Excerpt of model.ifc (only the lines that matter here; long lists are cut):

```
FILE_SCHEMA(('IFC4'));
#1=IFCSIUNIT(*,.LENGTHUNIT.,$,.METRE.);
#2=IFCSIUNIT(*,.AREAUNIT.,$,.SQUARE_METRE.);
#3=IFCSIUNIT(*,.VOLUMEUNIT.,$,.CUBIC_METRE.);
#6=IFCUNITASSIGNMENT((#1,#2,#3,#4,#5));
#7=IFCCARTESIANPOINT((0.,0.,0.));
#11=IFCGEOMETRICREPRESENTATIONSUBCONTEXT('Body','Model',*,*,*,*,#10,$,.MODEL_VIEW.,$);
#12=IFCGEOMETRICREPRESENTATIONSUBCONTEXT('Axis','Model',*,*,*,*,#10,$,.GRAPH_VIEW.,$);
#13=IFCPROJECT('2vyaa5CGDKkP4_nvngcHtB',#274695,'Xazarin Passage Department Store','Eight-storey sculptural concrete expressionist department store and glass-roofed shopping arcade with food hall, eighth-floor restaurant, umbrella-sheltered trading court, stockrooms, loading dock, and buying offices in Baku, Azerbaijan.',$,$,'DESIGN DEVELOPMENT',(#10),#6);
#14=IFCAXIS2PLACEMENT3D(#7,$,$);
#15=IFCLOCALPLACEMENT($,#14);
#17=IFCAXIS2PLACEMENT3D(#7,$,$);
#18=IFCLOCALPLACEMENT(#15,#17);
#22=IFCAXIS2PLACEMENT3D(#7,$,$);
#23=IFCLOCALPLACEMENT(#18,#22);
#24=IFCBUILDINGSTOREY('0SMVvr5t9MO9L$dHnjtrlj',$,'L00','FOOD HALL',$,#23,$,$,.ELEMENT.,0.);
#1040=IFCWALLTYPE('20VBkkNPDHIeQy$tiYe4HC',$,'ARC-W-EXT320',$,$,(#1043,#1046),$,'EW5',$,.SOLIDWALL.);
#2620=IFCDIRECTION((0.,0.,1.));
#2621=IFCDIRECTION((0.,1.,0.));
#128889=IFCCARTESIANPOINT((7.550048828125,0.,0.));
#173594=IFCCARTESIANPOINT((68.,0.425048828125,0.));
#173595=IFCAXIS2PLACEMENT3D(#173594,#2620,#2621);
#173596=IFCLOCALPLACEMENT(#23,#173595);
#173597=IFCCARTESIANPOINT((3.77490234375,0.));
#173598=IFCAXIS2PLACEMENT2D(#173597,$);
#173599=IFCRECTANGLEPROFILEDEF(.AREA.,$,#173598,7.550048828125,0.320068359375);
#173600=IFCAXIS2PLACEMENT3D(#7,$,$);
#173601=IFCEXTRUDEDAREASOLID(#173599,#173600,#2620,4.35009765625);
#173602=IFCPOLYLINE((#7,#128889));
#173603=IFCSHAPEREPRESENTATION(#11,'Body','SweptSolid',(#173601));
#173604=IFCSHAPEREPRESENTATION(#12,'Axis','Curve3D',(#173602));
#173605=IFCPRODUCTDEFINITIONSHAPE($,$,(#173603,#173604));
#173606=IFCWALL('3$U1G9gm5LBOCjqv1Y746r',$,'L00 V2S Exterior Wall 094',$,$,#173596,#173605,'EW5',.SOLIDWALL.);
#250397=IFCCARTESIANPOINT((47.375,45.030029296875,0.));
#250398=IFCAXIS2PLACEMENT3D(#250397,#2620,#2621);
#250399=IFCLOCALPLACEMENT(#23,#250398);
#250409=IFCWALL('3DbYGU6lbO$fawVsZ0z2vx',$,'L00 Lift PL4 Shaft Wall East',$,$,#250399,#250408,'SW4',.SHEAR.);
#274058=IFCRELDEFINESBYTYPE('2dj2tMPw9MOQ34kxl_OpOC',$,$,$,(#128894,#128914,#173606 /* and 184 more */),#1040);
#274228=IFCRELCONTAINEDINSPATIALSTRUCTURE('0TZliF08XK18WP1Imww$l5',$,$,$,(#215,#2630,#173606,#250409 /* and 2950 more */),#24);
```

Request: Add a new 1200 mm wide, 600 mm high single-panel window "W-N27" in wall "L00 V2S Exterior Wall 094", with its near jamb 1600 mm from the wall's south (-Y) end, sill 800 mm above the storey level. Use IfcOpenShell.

```python
import numpy as np
import ifcopenshell
import ifcopenshell.api.feature
import ifcopenshell.api.geometry
import ifcopenshell.api.root
import ifcopenshell.api.spatial
import ifcopenshell.geom
import ifcopenshell.util.element
import ifcopenshell.util.placement
import ifcopenshell.util.representation
import ifcopenshell.util.shape
import ifcopenshell.util.unit

model = ifcopenshell.open("model.ifc")
unit_scale = ifcopenshell.util.unit.calculate_unit_scale(model)
settings = ifcopenshell.geom.settings()


def volume(element):
    """Net volume in cubic metres, openings subtracted."""
    shape = ifcopenshell.geom.create_shape(settings, element)
    return ifcopenshell.util.shape.get_volume(shape.geometry)


wall = model.by_id(173606)
storey = ifcopenshell.util.element.get_container(wall, ifc_class="IfcBuildingStorey")
context = ifcopenshell.util.representation.get_context(model, "Model", "Body", "MODEL_VIEW")
before = volume(wall)

width, height, from_end, sill = 1.2, 0.6, 1.6, 0.8  # metres

# The wall runs along its own X axis, and the end named is its -X end.
wall_shape = ifcopenshell.geom.create_shape(settings, wall)
x, y, z = ifcopenshell.util.shape.get_vertices(wall_shape.geometry).T
start = x.min() + from_end
face, thickness = float(y.min()), float(y.max() - y.min())
wall_matrix = ifcopenshell.util.placement.get_local_placement(wall.ObjectPlacement)
level = ifcopenshell.util.placement.get_local_placement(storey.ObjectPlacement)[2, 3]


def in_wall(x, y):
    """Placement at x, y metres in the wall's axes, at sill height."""
    matrix = wall_matrix.copy()
    matrix[:, 3] = wall_matrix @ np.array([x / unit_scale, y / unit_scale, 0.0, 1.0])
    matrix[2, 3] = level + sill / unit_scale
    return matrix


# Opening: a box that overshoots both wall faces by 50 mm.
opening = ifcopenshell.api.root.create_entity(model, ifc_class="IfcOpeningElement", predefined_type="OPENING")
box = ifcopenshell.api.geometry.add_wall_representation(
    model, context=context, length=width, height=height, thickness=thickness + 0.1
)
ifcopenshell.api.geometry.assign_representation(model, product=opening, representation=box)
ifcopenshell.api.geometry.edit_object_placement(model, product=opening, matrix=in_wall(start, face - 0.05), is_si=False)
ifcopenshell.api.feature.add_feature(model, feature=opening, element=wall)

window = ifcopenshell.api.root.create_entity(model, ifc_class="IfcWindow", name="W-N27", predefined_type="WINDOW")
window.OverallWidth, window.OverallHeight = width / unit_scale, height / unit_scale
window.PartitioningType = "SINGLE_PANEL"
body = ifcopenshell.api.geometry.add_window_representation(
    model,
    context=context,
    overall_width=window.OverallWidth,
    overall_height=window.OverallHeight,
    partition_type="SINGLE_PANEL",
)
ifcopenshell.api.geometry.assign_representation(model, product=window, representation=body)
ifcopenshell.api.spatial.assign_container(model, products=[window], relating_structure=storey)
ifcopenshell.api.feature.add_filling(model, opening=opening, element=window)

# Centre the window in the wall's thickness.
ifcopenshell.api.geometry.edit_object_placement(model, product=window, matrix=in_wall(start, face), is_si=False)
window_shape = ifcopenshell.geom.create_shape(settings, window)
depth = ifcopenshell.util.shape.get_vertices(window_shape.geometry)[:, 1]
offset = face + thickness / 2 - (depth.min() + depth.max()) / 2
ifcopenshell.api.geometry.edit_object_placement(model, product=window, matrix=in_wall(start, offset), is_si=False)

after = volume(wall)

print(f"wall volume {before:.3f} -> {after:.3f} m3")

model.write("model_v2.ifc")
```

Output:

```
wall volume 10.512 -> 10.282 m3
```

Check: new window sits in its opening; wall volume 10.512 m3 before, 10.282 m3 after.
